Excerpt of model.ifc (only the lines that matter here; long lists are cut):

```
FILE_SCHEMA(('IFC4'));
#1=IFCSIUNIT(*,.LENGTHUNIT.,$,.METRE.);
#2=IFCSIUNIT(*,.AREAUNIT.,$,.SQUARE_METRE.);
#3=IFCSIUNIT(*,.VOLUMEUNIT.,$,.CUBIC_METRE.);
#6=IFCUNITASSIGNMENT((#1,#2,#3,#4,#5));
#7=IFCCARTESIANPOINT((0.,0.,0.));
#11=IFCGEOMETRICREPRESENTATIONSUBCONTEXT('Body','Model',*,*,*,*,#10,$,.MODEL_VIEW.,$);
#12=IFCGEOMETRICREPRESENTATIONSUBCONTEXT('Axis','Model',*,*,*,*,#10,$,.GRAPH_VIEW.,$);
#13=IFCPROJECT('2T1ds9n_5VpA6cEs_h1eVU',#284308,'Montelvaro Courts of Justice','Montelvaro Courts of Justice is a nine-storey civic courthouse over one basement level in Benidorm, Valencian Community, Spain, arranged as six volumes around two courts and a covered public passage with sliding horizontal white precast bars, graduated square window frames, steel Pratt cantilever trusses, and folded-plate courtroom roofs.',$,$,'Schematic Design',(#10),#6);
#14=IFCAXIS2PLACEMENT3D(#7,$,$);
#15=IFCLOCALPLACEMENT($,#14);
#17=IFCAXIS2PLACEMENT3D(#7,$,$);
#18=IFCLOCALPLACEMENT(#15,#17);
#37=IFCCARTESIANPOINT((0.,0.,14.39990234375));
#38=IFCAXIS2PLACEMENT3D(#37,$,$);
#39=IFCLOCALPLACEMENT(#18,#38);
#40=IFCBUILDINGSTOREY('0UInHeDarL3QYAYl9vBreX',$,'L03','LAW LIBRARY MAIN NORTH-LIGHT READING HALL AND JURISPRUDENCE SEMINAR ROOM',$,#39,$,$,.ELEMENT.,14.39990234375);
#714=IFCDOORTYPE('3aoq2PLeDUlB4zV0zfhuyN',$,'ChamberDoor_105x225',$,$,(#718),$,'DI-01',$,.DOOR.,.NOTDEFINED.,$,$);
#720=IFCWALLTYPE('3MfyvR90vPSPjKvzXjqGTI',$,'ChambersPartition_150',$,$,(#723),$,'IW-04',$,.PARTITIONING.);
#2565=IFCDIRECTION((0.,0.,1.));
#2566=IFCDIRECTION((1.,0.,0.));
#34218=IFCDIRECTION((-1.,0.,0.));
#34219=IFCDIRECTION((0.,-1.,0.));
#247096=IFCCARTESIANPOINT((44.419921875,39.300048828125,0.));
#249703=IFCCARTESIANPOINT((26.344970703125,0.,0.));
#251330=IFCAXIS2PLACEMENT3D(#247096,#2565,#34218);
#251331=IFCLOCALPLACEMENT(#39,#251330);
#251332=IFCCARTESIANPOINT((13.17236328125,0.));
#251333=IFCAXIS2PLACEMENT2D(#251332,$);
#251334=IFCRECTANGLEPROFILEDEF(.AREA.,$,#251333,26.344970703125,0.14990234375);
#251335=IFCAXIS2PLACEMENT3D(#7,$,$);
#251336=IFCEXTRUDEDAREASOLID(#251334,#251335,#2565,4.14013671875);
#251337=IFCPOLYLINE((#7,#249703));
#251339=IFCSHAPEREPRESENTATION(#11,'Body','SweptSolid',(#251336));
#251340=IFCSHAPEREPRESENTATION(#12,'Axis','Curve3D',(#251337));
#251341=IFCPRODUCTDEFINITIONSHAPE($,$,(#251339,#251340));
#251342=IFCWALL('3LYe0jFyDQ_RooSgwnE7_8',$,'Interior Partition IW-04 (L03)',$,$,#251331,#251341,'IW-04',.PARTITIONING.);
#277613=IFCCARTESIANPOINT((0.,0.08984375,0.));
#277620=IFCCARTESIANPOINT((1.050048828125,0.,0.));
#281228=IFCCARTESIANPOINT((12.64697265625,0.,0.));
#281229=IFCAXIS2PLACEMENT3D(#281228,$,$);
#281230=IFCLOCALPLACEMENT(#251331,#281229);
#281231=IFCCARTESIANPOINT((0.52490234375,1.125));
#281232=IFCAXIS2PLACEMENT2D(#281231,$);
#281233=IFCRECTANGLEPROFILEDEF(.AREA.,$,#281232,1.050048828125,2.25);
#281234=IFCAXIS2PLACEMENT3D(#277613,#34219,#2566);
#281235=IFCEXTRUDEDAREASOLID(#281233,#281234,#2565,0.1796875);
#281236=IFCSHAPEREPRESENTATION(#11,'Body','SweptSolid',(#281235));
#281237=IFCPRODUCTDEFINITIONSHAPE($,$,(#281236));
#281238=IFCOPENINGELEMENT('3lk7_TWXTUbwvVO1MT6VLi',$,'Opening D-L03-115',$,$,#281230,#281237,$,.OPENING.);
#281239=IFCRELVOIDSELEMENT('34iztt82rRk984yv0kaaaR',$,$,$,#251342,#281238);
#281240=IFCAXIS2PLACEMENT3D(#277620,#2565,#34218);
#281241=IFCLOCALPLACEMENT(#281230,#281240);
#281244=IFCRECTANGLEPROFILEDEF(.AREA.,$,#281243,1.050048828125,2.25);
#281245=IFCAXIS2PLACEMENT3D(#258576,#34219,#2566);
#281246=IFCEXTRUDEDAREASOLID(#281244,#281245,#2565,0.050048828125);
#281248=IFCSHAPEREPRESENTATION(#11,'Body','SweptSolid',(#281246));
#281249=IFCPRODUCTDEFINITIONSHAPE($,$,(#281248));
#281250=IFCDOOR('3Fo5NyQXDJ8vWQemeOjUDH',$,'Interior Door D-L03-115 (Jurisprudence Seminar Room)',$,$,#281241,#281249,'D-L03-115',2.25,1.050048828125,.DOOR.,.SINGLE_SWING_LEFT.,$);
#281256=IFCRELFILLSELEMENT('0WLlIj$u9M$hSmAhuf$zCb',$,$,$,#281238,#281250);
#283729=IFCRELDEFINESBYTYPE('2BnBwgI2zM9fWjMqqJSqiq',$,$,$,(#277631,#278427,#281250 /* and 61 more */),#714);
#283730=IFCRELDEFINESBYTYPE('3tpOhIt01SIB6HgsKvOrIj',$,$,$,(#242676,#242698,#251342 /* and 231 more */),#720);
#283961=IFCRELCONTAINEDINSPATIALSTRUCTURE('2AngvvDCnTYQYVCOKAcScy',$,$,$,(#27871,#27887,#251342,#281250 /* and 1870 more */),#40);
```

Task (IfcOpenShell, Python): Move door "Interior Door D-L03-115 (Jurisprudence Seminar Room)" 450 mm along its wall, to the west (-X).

```python
import ifcopenshell
import ifcopenshell.api.geometry
import ifcopenshell.util.placement
import ifcopenshell.util.unit

model = ifcopenshell.open("model.ifc")
unit_scale = ifcopenshell.util.unit.calculate_unit_scale(model)

door = model.by_id(281250)
opening = door.FillsVoids[0].RelatingOpeningElement
wall = opening.VoidsElements[0].RelatingBuildingElement

wall_matrix = ifcopenshell.util.placement.get_local_placement(wall.ObjectPlacement)
shift = wall_matrix[:3, 0] * 0.45 / unit_scale
before = ifcopenshell.util.placement.get_local_placement(door.ObjectPlacement)[:3, 3].copy()

# The door is placed relative to its opening, so it follows when the opening moves.
matrix = ifcopenshell.util.placement.get_local_placement(opening.ObjectPlacement)
matrix[:3, 3] += shift
ifcopenshell.api.geometry.edit_object_placement(
    model, product=opening, matrix=matrix, is_si=False, should_transform_children=True
)

after = ifcopenshell.util.placement.get_local_placement(door.ObjectPlacement)[:3, 3]
print("door moved by", (after - before).round(3) + 0.0)

model.write("model_edited.ifc")
```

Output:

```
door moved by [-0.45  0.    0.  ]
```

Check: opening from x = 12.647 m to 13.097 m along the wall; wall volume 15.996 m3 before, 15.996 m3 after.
